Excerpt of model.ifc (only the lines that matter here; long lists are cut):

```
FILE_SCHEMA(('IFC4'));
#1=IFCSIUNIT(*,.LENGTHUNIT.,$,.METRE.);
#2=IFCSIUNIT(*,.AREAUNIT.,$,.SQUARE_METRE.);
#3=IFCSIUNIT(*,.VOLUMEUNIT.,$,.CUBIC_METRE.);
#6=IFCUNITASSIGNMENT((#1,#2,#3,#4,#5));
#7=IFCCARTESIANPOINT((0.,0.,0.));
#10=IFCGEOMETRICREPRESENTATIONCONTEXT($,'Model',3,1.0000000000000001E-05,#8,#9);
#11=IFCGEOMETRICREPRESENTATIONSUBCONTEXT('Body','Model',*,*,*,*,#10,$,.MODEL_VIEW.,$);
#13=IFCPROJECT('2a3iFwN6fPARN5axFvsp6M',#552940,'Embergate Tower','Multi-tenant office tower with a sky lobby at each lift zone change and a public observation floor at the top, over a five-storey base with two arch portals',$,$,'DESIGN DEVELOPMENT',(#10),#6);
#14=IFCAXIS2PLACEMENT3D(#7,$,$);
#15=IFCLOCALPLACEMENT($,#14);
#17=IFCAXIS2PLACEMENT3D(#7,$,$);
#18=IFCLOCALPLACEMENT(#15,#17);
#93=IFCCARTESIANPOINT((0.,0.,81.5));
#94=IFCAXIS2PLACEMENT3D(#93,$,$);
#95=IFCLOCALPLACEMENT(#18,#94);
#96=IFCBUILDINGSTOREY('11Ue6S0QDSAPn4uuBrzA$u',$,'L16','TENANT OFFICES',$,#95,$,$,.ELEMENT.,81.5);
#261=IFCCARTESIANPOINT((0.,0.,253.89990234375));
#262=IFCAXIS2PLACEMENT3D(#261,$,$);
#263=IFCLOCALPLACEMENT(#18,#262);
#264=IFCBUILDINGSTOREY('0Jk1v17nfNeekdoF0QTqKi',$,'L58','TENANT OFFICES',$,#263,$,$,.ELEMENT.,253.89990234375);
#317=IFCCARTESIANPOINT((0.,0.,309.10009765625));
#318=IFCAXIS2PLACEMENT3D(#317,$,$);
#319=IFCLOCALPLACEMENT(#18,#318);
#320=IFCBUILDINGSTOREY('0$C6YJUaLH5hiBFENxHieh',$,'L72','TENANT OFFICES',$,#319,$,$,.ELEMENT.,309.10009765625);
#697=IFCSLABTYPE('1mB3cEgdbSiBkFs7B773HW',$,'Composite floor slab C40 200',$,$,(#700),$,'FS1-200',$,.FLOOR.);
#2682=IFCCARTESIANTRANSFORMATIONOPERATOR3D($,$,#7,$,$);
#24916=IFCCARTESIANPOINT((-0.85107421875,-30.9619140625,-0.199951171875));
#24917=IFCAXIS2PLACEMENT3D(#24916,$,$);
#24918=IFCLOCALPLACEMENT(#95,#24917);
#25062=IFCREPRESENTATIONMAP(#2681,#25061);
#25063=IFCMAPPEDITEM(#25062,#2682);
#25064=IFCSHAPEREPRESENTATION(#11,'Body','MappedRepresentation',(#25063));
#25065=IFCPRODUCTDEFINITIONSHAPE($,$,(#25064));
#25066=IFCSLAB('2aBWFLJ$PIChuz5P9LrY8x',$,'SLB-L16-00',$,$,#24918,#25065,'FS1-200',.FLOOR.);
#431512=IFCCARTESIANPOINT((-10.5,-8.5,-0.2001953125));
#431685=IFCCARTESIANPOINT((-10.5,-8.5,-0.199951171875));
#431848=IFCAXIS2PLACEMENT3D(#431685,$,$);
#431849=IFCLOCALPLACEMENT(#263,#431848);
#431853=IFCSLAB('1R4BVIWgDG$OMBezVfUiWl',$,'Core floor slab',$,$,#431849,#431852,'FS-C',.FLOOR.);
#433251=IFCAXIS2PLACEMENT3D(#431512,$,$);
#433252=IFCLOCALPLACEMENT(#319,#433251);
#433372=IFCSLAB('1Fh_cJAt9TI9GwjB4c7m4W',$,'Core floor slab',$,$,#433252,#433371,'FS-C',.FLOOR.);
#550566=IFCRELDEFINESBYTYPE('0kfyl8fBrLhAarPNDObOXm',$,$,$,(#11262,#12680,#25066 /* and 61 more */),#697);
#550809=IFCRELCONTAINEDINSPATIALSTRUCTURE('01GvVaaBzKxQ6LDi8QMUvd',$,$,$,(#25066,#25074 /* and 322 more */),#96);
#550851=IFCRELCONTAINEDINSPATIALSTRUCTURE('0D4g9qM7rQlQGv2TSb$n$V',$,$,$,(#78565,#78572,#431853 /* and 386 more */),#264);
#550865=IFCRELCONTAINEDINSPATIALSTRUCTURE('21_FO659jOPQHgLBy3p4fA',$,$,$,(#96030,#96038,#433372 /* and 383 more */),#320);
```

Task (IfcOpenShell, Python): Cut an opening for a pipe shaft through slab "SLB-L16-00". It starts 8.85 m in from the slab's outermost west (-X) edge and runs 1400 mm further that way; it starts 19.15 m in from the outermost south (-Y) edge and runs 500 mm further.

```python
import numpy as np
import ifcopenshell
import ifcopenshell.api.feature
import ifcopenshell.api.geometry
import ifcopenshell.api.root
import ifcopenshell.geom
import ifcopenshell.util.placement
import ifcopenshell.util.representation
import ifcopenshell.util.shape
import ifcopenshell.util.unit

model = ifcopenshell.open("model.ifc")
unit_scale = ifcopenshell.util.unit.calculate_unit_scale(model)
settings = ifcopenshell.geom.settings()


def volume(element):
    """Net volume in cubic metres, openings subtracted."""
    shape = ifcopenshell.geom.create_shape(settings, element)
    return ifcopenshell.util.shape.get_volume(shape.geometry)


slab = model.by_guid("2aBWFLJ$PIChuz5P9LrY8x")
before = volume(slab)

# Extent in the slab's own axes, in metres. The edges named are its -X and -Y sides.
slab_shape = ifcopenshell.geom.create_shape(settings, slab)
vertices = ifcopenshell.util.shape.get_vertices(slab_shape.geometry)
x_min, y_min, bottom = vertices.min(axis=0)
top = vertices[:, 2].max()

opening = ifcopenshell.api.root.create_entity(model, ifc_class="IfcOpeningElement", name="Pipe shaft opening", predefined_type="OPENING")
context = ifcopenshell.util.representation.get_context(model, "Model", "Body", "MODEL_VIEW")
width, depth = 1.4, 0.5
outline = [(0.0, 0.0), (width, 0.0), (width, depth), (0.0, depth), (0.0, 0.0)]
# Overshoot both faces by 50 mm so the cut is clean.
shape = ifcopenshell.api.geometry.add_slab_representation(
    model, context=context, depth=top - bottom + 0.1, polyline=outline
)
ifcopenshell.api.geometry.assign_representation(model, product=opening, representation=shape)

matrix = ifcopenshell.util.placement.get_local_placement(slab.ObjectPlacement)
matrix[:, 3] = matrix @ np.append(np.array([x_min + 8.85, y_min + 19.15, bottom - 0.05]) / unit_scale, 1.0)
ifcopenshell.api.geometry.edit_object_placement(model, product=opening, matrix=matrix, is_si=False)
ifcopenshell.api.feature.add_feature(model, feature=opening, element=slab)

after = volume(slab)

print(f"slab volume {before:.3f} -> {after:.3f} m3")

model.write("model_v2.ifc")
```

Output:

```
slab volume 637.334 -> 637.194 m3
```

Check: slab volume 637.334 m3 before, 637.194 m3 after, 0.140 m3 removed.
